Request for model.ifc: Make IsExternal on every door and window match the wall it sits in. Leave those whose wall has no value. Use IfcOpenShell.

First a look at what the model holds.

```python
import ifcopenshell
import ifcopenshell.util.element

model = ifcopenshell.open("model.ifc")
print(model.schema)
seen = {}
for e in model.by_type("IfcDoor") + model.by_type("IfcWindow"):
    if not e.FillsVoids:
        continue
    host = e.FillsVoids[0].RelatingOpeningElement.VoidsElements[0].RelatingBuildingElement
    own = ifcopenshell.util.element.get_pset(e, f"Pset_{e.is_a()[3:].removesuffix('StandardCase')}Common", "IsExternal")
    wall = ifcopenshell.util.element.get_pset(host, "Pset_WallCommon", "IsExternal")
    seen[e.is_a(), own, wall] = seen.get((e.is_a(), own, wall), 0) + 1
for (cls, own, wall), count in sorted(seen.items(), key=str):
    print(count, cls, "IsExternal:", own, "| host wall:", wall)
```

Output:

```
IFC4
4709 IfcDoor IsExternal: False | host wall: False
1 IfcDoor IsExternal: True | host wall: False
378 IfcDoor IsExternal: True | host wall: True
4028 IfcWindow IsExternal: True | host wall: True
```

```python
import ifcopenshell
import ifcopenshell.api.pset
import ifcopenshell.util.element

model = ifcopenshell.open("model.ifc")

count = 0
for ifc_class, pset_name in (("IfcDoor", "Pset_DoorCommon"), ("IfcWindow", "Pset_WindowCommon")):
    for e in model.by_type(ifc_class):
        if not e.FillsVoids:
            continue
        host = e.FillsVoids[0].RelatingOpeningElement.VoidsElements[0].RelatingBuildingElement
        external = ifcopenshell.util.element.get_pset(host, "Pset_WallCommon", "IsExternal")
        if external is None or ifcopenshell.util.element.get_pset(e, pset_name, "IsExternal") == external:
            continue
        pset = ifcopenshell.api.pset.add_pset(model, product=e, name=pset_name)
        ifcopenshell.api.pset.edit_pset(model, pset=pset, properties={"IsExternal": external})
        count += 1

print(count, "updated")

model.write("model_v2.ifc")
```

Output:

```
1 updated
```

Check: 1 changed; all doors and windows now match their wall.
